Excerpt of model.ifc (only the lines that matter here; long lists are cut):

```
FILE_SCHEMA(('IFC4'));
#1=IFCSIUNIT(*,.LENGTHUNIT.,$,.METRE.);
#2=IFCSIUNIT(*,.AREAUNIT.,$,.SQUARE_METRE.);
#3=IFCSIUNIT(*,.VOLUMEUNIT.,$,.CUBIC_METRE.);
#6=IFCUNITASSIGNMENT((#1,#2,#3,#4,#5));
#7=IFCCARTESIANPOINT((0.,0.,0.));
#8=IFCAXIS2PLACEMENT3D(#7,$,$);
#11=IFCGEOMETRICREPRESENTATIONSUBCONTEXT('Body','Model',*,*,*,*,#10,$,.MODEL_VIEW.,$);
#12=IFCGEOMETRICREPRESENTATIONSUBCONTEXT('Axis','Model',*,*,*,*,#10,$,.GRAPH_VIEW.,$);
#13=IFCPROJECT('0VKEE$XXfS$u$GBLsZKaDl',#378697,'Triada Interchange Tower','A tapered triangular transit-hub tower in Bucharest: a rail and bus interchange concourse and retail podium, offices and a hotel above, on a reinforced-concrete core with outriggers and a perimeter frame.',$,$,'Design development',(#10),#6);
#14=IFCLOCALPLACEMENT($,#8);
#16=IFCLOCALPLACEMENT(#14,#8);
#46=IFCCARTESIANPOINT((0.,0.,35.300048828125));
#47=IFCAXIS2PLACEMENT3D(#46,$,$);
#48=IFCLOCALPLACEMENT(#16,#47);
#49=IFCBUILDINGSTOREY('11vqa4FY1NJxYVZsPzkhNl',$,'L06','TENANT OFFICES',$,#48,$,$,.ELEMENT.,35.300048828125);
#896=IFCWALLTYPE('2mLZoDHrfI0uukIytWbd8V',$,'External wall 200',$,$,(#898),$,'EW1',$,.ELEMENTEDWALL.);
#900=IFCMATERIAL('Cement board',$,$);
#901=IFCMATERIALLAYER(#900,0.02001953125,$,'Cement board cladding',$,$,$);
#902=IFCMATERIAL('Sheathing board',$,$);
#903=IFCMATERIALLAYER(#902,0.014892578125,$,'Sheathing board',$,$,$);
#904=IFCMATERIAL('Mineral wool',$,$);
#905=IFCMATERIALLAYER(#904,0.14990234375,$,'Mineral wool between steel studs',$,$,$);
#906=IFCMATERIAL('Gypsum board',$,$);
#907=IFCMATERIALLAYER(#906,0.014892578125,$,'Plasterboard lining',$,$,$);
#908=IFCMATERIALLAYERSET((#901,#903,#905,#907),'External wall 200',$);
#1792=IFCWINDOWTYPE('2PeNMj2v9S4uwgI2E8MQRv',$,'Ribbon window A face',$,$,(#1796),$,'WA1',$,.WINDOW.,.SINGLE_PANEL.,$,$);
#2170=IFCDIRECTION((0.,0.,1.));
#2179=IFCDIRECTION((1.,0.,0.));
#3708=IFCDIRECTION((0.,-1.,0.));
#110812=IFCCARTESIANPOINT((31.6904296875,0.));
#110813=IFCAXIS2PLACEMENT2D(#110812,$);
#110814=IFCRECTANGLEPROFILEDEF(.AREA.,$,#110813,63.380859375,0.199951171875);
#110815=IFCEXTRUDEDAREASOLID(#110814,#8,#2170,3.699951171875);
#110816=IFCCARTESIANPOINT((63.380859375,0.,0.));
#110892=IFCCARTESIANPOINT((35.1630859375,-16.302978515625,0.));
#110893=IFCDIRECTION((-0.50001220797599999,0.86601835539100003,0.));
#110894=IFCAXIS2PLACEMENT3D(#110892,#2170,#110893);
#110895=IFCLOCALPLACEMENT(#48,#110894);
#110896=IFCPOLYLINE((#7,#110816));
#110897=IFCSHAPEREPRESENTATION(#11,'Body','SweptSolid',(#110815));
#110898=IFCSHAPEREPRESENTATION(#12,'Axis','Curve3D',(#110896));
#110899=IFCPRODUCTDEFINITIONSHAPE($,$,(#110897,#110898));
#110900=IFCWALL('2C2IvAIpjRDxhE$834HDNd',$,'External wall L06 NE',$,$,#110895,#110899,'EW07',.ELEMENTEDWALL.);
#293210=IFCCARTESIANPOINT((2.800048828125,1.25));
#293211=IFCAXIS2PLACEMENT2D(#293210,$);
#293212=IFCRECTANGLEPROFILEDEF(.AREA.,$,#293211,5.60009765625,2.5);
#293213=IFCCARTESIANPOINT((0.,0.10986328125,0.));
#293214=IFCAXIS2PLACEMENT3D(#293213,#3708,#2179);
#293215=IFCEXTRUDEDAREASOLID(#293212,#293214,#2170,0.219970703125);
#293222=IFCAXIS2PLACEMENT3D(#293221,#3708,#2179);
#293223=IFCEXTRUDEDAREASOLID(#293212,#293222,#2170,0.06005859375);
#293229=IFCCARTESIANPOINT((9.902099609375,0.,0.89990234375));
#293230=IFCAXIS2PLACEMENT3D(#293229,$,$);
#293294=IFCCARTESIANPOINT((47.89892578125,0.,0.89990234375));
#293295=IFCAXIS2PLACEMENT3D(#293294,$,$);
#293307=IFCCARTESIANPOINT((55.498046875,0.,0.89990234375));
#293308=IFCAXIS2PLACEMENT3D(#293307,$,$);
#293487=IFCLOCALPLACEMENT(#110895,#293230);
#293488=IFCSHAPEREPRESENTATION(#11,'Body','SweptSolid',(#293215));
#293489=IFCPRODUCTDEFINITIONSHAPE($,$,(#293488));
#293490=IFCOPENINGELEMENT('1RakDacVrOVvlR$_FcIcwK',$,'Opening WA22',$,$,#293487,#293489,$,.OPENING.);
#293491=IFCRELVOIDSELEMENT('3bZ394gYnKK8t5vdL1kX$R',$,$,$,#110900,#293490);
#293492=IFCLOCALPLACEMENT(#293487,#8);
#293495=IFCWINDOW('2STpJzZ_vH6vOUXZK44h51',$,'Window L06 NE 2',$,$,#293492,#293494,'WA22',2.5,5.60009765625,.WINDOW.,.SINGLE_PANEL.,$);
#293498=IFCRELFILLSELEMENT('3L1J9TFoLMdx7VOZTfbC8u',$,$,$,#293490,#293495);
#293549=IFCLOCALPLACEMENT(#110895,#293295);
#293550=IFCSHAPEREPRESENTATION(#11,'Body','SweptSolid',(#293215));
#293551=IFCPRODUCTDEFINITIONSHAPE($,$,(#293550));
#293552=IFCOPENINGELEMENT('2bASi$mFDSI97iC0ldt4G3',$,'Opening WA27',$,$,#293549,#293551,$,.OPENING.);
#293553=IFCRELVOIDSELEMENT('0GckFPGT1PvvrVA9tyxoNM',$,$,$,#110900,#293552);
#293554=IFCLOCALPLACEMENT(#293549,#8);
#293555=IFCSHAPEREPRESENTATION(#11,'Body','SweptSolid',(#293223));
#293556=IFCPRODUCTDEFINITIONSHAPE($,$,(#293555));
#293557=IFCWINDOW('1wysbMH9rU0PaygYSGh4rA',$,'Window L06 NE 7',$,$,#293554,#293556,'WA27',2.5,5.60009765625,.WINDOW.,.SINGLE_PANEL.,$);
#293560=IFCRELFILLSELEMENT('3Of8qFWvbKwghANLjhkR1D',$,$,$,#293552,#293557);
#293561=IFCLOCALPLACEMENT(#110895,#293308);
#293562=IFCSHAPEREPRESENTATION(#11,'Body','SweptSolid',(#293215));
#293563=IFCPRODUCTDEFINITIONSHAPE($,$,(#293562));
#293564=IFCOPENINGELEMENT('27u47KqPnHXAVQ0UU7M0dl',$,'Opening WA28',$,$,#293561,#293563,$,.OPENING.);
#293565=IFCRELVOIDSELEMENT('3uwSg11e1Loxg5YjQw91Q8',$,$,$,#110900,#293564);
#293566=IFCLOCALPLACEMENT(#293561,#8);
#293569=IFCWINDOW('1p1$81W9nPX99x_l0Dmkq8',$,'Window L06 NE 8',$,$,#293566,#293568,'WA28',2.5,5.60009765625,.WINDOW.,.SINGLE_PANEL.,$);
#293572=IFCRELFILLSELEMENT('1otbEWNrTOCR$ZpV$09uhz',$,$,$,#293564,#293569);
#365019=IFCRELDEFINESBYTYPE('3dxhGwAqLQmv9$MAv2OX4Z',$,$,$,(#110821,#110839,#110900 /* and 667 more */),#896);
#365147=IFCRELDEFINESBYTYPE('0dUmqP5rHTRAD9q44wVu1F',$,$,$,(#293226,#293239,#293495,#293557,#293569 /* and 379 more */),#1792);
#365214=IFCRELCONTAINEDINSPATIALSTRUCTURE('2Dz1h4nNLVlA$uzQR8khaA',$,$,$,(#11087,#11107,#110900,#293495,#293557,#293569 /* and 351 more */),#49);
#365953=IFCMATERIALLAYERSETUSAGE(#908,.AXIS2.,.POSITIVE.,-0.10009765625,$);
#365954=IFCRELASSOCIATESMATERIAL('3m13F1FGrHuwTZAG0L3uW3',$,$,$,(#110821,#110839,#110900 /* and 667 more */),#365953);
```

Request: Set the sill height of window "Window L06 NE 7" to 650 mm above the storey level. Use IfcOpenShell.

```python
import numpy as np
import ifcopenshell
import ifcopenshell.api.geometry
import ifcopenshell.geom
import ifcopenshell.util.element
import ifcopenshell.util.placement
import ifcopenshell.util.shape
import ifcopenshell.util.unit

model = ifcopenshell.open("model.ifc")
unit_scale = ifcopenshell.util.unit.calculate_unit_scale(model)

window = model.by_guid("1wysbMH9rU0PaygYSGh4rA")
opening = window.FillsVoids[0].RelatingOpeningElement
storey = ifcopenshell.util.element.get_container(window, ifc_class="IfcBuildingStorey")
level = ifcopenshell.util.placement.get_local_placement(storey.ObjectPlacement)[2, 3]

# The opening's origin need not be at the sill, so measure its lowest point.
shape = ifcopenshell.geom.create_shape(ifcopenshell.geom.settings(), opening)
bottom = ifcopenshell.util.shape.get_shape_bottom_elevation(shape, shape.geometry) / unit_scale
dz = level + 0.65 / unit_scale - bottom

shift = np.array([0.0, 0.0, dz])
# The window is placed relative to its opening, so it follows when the opening moves.
matrix = ifcopenshell.util.placement.get_local_placement(opening.ObjectPlacement)
matrix[:3, 3] += shift
ifcopenshell.api.geometry.edit_object_placement(
    model, product=opening, matrix=matrix, is_si=False, should_transform_children=True
)

print(f"moved by {dz * unit_scale:+.3f} m")

model.write("model_rev.ifc")
```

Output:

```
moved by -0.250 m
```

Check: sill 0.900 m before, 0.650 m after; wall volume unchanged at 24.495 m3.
